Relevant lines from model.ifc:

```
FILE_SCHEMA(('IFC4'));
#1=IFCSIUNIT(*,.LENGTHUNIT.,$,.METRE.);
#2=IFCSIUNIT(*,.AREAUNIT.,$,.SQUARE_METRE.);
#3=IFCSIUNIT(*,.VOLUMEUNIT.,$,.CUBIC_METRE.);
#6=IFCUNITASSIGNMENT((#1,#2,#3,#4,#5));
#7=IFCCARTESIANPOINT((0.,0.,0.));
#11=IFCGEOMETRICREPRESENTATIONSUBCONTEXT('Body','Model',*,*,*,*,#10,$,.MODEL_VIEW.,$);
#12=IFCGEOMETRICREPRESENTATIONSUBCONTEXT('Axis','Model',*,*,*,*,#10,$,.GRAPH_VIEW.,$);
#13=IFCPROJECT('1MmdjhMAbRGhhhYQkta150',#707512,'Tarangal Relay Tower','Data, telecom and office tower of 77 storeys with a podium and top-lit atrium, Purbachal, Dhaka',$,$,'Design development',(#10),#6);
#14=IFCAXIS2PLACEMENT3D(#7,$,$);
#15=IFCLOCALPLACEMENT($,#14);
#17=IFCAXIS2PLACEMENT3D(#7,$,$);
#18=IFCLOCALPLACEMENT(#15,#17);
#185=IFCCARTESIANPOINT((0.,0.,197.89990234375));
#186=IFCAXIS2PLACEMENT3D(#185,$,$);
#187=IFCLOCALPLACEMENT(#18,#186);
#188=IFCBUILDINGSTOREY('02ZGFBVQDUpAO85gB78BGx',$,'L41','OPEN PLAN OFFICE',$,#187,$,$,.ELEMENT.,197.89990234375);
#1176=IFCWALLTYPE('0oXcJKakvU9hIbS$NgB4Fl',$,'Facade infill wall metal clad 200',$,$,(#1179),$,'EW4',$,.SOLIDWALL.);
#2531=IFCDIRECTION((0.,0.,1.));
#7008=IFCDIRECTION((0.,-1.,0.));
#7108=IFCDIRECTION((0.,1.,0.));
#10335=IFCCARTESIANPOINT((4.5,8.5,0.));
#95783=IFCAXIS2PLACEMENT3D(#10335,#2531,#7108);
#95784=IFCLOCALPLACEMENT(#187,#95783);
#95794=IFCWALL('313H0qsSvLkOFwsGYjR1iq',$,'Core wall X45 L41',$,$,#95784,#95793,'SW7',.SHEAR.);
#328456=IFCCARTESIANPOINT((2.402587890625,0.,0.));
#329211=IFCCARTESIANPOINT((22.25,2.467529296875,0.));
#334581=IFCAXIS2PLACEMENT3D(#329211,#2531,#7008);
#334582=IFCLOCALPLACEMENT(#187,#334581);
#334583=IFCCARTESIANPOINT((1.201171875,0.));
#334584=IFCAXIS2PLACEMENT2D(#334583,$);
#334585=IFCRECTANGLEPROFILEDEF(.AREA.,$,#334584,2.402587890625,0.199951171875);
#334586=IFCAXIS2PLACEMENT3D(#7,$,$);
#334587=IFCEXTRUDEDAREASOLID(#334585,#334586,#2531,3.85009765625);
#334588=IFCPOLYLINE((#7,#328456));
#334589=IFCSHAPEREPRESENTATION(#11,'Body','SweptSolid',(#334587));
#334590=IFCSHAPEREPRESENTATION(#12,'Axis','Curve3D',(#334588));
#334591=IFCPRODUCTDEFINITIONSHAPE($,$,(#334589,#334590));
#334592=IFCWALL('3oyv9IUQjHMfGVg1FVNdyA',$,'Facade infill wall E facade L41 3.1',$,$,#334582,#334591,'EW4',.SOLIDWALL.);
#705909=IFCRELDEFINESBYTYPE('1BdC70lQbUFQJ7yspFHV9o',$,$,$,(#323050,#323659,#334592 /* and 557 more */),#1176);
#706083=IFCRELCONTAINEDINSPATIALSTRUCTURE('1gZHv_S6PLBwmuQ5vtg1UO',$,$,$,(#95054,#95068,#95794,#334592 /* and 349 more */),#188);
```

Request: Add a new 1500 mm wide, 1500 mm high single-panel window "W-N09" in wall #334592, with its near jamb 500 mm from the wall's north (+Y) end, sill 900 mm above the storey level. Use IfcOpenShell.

```python
import numpy as np
import ifcopenshell
import ifcopenshell.api.feature
import ifcopenshell.api.geometry
import ifcopenshell.api.root
import ifcopenshell.api.spatial
import ifcopenshell.geom
import ifcopenshell.util.element
import ifcopenshell.util.placement
import ifcopenshell.util.representation
import ifcopenshell.util.shape
import ifcopenshell.util.unit

model = ifcopenshell.open("model.ifc")
unit_scale = ifcopenshell.util.unit.calculate_unit_scale(model)
settings = ifcopenshell.geom.settings()


def volume(element):
    """Net volume in cubic metres, openings subtracted."""
    shape = ifcopenshell.geom.create_shape(settings, element)
    return ifcopenshell.util.shape.get_volume(shape.geometry)


wall = model.by_id(334592)
storey = ifcopenshell.util.element.get_container(wall, ifc_class="IfcBuildingStorey")
context = ifcopenshell.util.representation.get_context(model, "Model", "Body", "MODEL_VIEW")
before = volume(wall)

width, height, from_end, sill = 1.5, 1.5, 0.5, 0.9  # metres

# The wall runs along its own X axis, and the end named is its -X end.
wall_shape = ifcopenshell.geom.create_shape(settings, wall)
x, y, z = ifcopenshell.util.shape.get_vertices(wall_shape.geometry).T
start = x.min() + from_end
face, thickness = float(y.min()), float(y.max() - y.min())
wall_matrix = ifcopenshell.util.placement.get_local_placement(wall.ObjectPlacement)
level = ifcopenshell.util.placement.get_local_placement(storey.ObjectPlacement)[2, 3]


def in_wall(x, y):
    """Placement at x, y metres in the wall's axes, at sill height."""
    matrix = wall_matrix.copy()
    matrix[:, 3] = wall_matrix @ np.array([x / unit_scale, y / unit_scale, 0.0, 1.0])
    matrix[2, 3] = level + sill / unit_scale
    return matrix


# Opening: a box that overshoots both wall faces by 50 mm.
opening = ifcopenshell.api.root.create_entity(model, ifc_class="IfcOpeningElement", predefined_type="OPENING")
box = ifcopenshell.api.geometry.add_wall_representation(
    model, context=context, length=width, height=height, thickness=thickness + 0.1
)
ifcopenshell.api.geometry.assign_representation(model, product=opening, representation=box)
ifcopenshell.api.geometry.edit_object_placement(model, product=opening, matrix=in_wall(start, face - 0.05), is_si=False)
ifcopenshell.api.feature.add_feature(model, feature=opening, element=wall)

window = ifcopenshell.api.root.create_entity(model, ifc_class="IfcWindow", name="W-N09", predefined_type="WINDOW")
window.OverallWidth, window.OverallHeight = width / unit_scale, height / unit_scale
window.PartitioningType = "SINGLE_PANEL"
body = ifcopenshell.api.geometry.add_window_representation(
    model,
    context=context,
    overall_width=window.OverallWidth,
    overall_height=window.OverallHeight,
    partition_type="SINGLE_PANEL",
)
ifcopenshell.api.geometry.assign_representation(model, product=window, representation=body)
ifcopenshell.api.spatial.assign_container(model, products=[window], relating_structure=storey)
ifcopenshell.api.feature.add_filling(model, opening=opening, element=window)

# Centre the window in the wall's thickness.
ifcopenshell.api.geometry.edit_object_placement(model, product=window, matrix=in_wall(start, face), is_si=False)
window_shape = ifcopenshell.geom.create_shape(settings, window)
depth = ifcopenshell.util.shape.get_vertices(window_shape.geometry)[:, 1]
offset = face + thickness / 2 - (depth.min() + depth.max()) / 2
ifcopenshell.api.geometry.edit_object_placement(model, product=window, matrix=in_wall(start, offset), is_si=False)

after = volume(wall)

print(f"wall volume {before:.3f} -> {after:.3f} m3")

model.write("model_rev.ifc")
```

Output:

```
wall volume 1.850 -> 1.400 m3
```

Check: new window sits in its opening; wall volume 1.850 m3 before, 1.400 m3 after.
